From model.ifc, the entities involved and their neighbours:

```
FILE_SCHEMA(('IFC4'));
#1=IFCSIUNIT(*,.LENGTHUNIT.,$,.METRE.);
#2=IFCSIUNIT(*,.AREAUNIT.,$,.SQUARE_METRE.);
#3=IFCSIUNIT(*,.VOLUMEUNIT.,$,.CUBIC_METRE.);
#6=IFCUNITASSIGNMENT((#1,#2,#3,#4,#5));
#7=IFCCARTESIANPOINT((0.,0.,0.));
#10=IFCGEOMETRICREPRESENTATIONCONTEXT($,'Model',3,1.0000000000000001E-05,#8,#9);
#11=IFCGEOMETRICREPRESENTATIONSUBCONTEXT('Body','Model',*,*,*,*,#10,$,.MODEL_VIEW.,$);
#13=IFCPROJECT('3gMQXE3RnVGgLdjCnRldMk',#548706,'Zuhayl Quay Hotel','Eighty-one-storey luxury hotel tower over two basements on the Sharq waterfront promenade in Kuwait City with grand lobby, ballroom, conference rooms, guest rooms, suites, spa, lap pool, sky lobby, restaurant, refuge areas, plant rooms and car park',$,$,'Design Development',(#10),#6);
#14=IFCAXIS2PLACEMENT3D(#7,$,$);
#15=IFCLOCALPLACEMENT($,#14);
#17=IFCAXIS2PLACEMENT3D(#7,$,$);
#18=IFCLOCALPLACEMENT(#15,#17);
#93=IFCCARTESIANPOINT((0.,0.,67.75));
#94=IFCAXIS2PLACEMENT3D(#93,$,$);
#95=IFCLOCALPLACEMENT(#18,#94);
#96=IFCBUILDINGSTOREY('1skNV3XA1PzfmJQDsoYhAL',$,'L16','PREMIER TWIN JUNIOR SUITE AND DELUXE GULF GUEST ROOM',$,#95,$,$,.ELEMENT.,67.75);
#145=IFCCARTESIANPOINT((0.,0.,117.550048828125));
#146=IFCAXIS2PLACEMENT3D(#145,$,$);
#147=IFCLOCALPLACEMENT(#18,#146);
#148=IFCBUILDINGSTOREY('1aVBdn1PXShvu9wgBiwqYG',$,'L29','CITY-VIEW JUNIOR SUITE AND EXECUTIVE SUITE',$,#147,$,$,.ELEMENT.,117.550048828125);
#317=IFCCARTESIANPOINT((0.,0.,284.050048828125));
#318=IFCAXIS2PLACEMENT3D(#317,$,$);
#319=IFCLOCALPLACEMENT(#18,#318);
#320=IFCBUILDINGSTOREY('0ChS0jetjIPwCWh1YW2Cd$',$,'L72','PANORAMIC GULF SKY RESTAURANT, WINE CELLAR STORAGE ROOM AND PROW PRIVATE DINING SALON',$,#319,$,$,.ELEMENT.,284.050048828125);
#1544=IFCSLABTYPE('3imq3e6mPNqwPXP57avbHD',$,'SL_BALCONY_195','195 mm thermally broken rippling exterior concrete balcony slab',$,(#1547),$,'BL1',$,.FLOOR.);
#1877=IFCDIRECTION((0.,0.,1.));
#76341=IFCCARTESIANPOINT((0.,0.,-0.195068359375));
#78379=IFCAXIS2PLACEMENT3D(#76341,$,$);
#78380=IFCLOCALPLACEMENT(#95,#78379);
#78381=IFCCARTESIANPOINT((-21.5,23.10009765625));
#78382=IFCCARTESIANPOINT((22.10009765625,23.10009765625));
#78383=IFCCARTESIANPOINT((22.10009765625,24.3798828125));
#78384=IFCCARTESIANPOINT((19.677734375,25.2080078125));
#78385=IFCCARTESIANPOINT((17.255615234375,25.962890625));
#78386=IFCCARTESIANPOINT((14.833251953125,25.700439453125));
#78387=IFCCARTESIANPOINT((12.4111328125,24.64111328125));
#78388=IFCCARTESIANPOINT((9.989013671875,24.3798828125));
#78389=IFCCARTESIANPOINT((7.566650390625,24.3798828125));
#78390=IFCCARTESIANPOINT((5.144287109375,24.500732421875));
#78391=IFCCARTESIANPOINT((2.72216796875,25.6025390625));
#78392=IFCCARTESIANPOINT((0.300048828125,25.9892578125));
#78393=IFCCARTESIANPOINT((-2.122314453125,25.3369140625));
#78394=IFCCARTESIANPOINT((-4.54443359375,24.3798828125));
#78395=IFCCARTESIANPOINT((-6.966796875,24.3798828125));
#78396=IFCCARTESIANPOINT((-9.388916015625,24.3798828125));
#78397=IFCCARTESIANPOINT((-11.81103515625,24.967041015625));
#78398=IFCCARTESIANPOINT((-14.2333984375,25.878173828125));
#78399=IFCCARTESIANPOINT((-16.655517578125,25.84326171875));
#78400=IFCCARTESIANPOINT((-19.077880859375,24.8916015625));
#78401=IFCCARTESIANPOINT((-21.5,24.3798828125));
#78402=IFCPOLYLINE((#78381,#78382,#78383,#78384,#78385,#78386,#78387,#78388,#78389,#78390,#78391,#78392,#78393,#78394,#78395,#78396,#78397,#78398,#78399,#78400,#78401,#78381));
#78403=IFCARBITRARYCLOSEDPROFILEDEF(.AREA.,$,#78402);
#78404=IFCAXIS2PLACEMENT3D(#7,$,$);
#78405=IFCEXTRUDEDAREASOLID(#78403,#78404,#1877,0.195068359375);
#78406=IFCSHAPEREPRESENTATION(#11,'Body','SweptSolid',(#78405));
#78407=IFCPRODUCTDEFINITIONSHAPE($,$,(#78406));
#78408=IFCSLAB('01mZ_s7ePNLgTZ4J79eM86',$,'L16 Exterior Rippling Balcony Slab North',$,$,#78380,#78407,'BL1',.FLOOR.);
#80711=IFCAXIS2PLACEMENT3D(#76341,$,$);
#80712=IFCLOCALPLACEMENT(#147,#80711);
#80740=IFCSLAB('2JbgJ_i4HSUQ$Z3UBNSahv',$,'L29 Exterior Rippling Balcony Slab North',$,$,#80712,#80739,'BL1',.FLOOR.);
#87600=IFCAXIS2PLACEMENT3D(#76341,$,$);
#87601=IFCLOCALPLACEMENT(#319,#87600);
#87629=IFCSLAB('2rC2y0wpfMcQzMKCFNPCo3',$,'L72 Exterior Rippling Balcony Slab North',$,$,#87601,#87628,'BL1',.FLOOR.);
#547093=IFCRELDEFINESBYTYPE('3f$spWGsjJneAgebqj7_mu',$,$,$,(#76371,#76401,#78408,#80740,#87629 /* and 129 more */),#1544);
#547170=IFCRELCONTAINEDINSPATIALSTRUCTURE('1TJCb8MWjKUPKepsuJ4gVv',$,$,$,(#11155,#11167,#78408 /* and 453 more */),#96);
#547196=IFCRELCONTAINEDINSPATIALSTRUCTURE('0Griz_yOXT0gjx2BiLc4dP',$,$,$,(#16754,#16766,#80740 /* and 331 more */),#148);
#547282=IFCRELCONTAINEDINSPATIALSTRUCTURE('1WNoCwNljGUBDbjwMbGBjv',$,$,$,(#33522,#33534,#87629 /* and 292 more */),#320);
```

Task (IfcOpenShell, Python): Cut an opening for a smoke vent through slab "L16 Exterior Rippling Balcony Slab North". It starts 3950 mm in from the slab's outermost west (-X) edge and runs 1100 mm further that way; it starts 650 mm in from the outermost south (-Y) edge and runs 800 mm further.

```python
import numpy as np
import ifcopenshell
import ifcopenshell.api.feature
import ifcopenshell.api.geometry
import ifcopenshell.api.root
import ifcopenshell.geom
import ifcopenshell.util.placement
import ifcopenshell.util.representation
import ifcopenshell.util.shape
import ifcopenshell.util.unit

model = ifcopenshell.open("model.ifc")
unit_scale = ifcopenshell.util.unit.calculate_unit_scale(model)
settings = ifcopenshell.geom.settings()


def volume(element):
    """Net volume in cubic metres, openings subtracted."""
    shape = ifcopenshell.geom.create_shape(settings, element)
    return ifcopenshell.util.shape.get_volume(shape.geometry)


slab = model.by_guid("01mZ_s7ePNLgTZ4J79eM86")
before = volume(slab)

# Extent in the slab's own axes, in metres. The edges named are its -X and -Y sides.
slab_shape = ifcopenshell.geom.create_shape(settings, slab)
vertices = ifcopenshell.util.shape.get_vertices(slab_shape.geometry)
x_min, y_min, bottom = vertices.min(axis=0)
top = vertices[:, 2].max()

opening = ifcopenshell.api.root.create_entity(model, ifc_class="IfcOpeningElement", name="Smoke vent opening", predefined_type="OPENING")
context = ifcopenshell.util.representation.get_context(model, "Model", "Body", "MODEL_VIEW")
width, depth = 1.1, 0.8
outline = [(0.0, 0.0), (width, 0.0), (width, depth), (0.0, depth), (0.0, 0.0)]
# Overshoot both faces by 50 mm so the cut is clean.
shape = ifcopenshell.api.geometry.add_slab_representation(
    model, context=context, depth=top - bottom + 0.1, polyline=outline
)
ifcopenshell.api.geometry.assign_representation(model, product=opening, representation=shape)

matrix = ifcopenshell.util.placement.get_local_placement(slab.ObjectPlacement)
matrix[:, 3] = matrix @ np.append(np.array([x_min + 3.95, y_min + 0.65, bottom - 0.05]) / unit_scale, 1.0)
ifcopenshell.api.geometry.edit_object_placement(model, product=opening, matrix=matrix, is_si=False)
ifcopenshell.api.feature.add_feature(model, feature=opening, element=slab)

after = volume(slab)

print(f"slab volume {before:.3f} -> {after:.3f} m3")

model.write("model-out.ifc")
```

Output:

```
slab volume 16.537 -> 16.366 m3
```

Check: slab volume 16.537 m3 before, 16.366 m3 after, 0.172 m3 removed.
